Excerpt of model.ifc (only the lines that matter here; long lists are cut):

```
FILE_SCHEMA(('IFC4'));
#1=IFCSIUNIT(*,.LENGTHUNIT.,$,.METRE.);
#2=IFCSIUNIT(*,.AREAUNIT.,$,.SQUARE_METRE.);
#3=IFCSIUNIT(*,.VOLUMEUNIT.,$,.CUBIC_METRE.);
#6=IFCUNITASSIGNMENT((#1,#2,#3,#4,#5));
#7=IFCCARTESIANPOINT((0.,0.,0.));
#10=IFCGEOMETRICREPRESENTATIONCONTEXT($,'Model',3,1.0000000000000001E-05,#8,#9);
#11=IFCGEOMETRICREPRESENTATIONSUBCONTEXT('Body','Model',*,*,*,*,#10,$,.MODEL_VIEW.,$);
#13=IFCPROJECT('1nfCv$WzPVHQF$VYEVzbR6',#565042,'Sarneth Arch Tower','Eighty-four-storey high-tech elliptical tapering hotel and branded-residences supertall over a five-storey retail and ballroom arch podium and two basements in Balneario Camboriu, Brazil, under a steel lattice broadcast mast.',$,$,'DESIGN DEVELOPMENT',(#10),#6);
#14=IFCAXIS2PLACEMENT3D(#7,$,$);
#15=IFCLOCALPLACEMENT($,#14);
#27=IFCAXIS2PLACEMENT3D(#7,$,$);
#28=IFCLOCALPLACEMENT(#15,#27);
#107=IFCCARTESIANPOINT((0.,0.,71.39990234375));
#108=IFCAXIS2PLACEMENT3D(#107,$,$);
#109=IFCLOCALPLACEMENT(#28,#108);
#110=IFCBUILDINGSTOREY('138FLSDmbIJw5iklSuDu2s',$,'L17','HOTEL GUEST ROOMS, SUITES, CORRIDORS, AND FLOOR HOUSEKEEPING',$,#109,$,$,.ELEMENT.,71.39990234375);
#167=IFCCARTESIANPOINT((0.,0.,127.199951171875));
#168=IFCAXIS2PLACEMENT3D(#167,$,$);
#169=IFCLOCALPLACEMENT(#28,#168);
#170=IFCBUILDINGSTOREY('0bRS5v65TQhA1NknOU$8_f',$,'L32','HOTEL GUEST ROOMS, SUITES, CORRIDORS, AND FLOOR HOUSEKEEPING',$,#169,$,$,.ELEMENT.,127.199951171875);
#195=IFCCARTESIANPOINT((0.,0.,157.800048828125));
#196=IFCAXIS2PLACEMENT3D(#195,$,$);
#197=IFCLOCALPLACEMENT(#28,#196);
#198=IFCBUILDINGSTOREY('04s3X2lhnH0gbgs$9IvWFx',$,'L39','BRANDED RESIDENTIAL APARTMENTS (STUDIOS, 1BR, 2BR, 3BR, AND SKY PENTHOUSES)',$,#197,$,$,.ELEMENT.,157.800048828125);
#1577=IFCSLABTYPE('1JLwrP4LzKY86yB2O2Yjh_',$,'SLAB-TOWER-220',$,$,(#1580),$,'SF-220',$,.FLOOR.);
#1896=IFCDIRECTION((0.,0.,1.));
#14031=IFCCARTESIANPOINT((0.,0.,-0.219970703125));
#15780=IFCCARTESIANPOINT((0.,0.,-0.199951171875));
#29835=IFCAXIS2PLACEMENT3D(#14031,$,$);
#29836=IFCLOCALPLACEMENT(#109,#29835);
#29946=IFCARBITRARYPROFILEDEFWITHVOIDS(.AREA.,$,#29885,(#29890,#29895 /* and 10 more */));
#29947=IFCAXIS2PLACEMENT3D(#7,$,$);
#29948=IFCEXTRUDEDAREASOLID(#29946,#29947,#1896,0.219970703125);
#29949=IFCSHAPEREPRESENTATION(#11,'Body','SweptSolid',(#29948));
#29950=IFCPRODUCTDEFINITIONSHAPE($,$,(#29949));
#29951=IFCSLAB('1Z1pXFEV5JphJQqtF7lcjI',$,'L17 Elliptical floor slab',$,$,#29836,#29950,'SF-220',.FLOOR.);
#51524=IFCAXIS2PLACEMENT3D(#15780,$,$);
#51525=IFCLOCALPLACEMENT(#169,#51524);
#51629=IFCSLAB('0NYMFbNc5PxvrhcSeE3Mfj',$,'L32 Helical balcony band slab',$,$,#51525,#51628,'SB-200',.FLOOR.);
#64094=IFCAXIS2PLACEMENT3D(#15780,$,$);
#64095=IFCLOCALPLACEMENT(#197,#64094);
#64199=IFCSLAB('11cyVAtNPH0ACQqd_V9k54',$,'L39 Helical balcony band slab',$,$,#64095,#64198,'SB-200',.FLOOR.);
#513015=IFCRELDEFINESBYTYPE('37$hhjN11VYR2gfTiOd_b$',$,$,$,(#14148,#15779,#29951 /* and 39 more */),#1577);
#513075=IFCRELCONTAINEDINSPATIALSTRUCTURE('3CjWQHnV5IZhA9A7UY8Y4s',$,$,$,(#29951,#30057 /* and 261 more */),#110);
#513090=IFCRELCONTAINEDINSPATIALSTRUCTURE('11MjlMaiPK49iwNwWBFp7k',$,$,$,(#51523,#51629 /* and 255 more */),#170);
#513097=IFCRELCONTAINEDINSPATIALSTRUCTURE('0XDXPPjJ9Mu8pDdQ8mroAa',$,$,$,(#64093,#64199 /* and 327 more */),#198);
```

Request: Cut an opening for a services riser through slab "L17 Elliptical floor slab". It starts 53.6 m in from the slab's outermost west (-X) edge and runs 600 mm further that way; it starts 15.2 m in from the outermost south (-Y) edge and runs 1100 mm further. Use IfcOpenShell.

```python
import numpy as np
import ifcopenshell
import ifcopenshell.api.feature
import ifcopenshell.api.geometry
import ifcopenshell.api.root
import ifcopenshell.geom
import ifcopenshell.util.placement
import ifcopenshell.util.representation
import ifcopenshell.util.shape
import ifcopenshell.util.unit

model = ifcopenshell.open("model.ifc")
unit_scale = ifcopenshell.util.unit.calculate_unit_scale(model)
settings = ifcopenshell.geom.settings()


def volume(element):
    """Net volume in cubic metres, openings subtracted."""
    shape = ifcopenshell.geom.create_shape(settings, element)
    return ifcopenshell.util.shape.get_volume(shape.geometry)


slab = model.by_guid("1Z1pXFEV5JphJQqtF7lcjI")
before = volume(slab)

# Extent in the slab's own axes, in metres. The edges named are its -X and -Y sides.
slab_shape = ifcopenshell.geom.create_shape(settings, slab)
vertices = ifcopenshell.util.shape.get_vertices(slab_shape.geometry)
x_min, y_min, bottom = vertices.min(axis=0)
top = vertices[:, 2].max()

opening = ifcopenshell.api.root.create_entity(model, ifc_class="IfcOpeningElement", name="Services riser opening", predefined_type="OPENING")
context = ifcopenshell.util.representation.get_context(model, "Model", "Body", "MODEL_VIEW")
width, depth = 0.6, 1.1
outline = [(0.0, 0.0), (width, 0.0), (width, depth), (0.0, depth), (0.0, 0.0)]
# Overshoot both faces by 50 mm so the cut is clean.
shape = ifcopenshell.api.geometry.add_slab_representation(
    model, context=context, depth=top - bottom + 0.1, polyline=outline
)
ifcopenshell.api.geometry.assign_representation(model, product=opening, representation=shape)

matrix = ifcopenshell.util.placement.get_local_placement(slab.ObjectPlacement)
matrix[:, 3] = matrix @ np.append(np.array([x_min + 53.6, y_min + 15.2, bottom - 0.05]) / unit_scale, 1.0)
ifcopenshell.api.geometry.edit_object_placement(model, product=opening, matrix=matrix, is_si=False)
ifcopenshell.api.feature.add_feature(model, feature=opening, element=slab)

after = volume(slab)

print(f"slab volume {before:.3f} -> {after:.3f} m3")

model.write("model_updated.ifc")
```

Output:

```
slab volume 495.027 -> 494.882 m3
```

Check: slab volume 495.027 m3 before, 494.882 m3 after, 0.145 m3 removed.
